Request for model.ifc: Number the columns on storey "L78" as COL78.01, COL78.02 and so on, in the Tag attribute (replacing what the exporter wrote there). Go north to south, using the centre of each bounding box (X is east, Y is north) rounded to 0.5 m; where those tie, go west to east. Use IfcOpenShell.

First a look at what the model holds.

```python
import ifcopenshell
import ifcopenshell.util.element
import ifcopenshell.util.placement

model = ifcopenshell.open("model.ifc")
print(model.schema)
storey = next(s for s in model.by_type("IfcBuildingStorey") if s.Name == "L78")
columns = [e for e in ifcopenshell.util.element.get_decomposition(storey) if e.is_a("IfcColumn")]
for e in sorted(columns, key=lambda e: e.id()):
    origin = ifcopenshell.util.placement.get_local_placement(e.ObjectPlacement)[:3, 3]
    print(e.id(), e.Tag, e.Name, origin.round(2) + 0.0, sep=" | ")
```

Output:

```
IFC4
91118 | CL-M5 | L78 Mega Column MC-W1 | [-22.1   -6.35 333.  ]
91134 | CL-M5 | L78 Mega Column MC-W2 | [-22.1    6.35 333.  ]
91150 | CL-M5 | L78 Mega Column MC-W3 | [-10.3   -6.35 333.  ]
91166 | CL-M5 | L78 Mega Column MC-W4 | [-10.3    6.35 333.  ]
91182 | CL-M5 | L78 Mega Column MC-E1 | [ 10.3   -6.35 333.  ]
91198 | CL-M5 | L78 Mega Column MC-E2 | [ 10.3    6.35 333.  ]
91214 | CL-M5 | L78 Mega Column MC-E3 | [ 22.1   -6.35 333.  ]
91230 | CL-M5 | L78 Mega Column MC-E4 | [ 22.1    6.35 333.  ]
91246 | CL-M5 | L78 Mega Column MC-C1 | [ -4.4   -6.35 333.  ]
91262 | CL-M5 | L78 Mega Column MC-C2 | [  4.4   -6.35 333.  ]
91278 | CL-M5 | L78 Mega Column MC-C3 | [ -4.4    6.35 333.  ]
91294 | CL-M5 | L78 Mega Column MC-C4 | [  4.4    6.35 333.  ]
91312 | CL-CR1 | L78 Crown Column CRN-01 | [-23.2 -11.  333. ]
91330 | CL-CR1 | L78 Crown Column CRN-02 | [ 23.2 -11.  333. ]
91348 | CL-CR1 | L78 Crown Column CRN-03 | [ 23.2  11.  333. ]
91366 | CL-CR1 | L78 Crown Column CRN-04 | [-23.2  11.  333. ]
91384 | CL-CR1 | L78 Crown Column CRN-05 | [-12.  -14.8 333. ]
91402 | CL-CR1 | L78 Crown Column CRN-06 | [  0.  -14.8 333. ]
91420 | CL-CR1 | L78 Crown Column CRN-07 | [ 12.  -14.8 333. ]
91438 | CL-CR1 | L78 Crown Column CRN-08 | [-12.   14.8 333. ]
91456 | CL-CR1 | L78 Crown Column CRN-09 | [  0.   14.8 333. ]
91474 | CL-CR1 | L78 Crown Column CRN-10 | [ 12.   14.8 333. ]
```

```python
import ifcopenshell
import ifcopenshell.geom
import ifcopenshell.util.element
import ifcopenshell.util.shape

model = ifcopenshell.open("model.ifc")
settings = ifcopenshell.geom.settings()
settings.set("use-world-coords", True)


def centre(element):
    shape = ifcopenshell.geom.create_shape(settings, element)
    return ifcopenshell.util.shape.get_bbox_centroid(shape.geometry)


storey = next(s for s in model.by_type("IfcBuildingStorey") if s.Name == "L78")
columns = [e for e in ifcopenshell.util.element.get_decomposition(storey) if e.is_a("IfcColumn")]

# Insertion points can sit at a corner or the storey origin, so sort by the geometry (in metres).
centres = {e: centre(e) for e in columns}
columns.sort(key=lambda e: (-round(centres[e][1] / 0.5), centres[e][0]))

for i, e in enumerate(columns, start=1):
    number = f"COL78.{i:02d}"
    e.Tag = number
    print(e.id(), number)

model.write("model_rev.ifc")
```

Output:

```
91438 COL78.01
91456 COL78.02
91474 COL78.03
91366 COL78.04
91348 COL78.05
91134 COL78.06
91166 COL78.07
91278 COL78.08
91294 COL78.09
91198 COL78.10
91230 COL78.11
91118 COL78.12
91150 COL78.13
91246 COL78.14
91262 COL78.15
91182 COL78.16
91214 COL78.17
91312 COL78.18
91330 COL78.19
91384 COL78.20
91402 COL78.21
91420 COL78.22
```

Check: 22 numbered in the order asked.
